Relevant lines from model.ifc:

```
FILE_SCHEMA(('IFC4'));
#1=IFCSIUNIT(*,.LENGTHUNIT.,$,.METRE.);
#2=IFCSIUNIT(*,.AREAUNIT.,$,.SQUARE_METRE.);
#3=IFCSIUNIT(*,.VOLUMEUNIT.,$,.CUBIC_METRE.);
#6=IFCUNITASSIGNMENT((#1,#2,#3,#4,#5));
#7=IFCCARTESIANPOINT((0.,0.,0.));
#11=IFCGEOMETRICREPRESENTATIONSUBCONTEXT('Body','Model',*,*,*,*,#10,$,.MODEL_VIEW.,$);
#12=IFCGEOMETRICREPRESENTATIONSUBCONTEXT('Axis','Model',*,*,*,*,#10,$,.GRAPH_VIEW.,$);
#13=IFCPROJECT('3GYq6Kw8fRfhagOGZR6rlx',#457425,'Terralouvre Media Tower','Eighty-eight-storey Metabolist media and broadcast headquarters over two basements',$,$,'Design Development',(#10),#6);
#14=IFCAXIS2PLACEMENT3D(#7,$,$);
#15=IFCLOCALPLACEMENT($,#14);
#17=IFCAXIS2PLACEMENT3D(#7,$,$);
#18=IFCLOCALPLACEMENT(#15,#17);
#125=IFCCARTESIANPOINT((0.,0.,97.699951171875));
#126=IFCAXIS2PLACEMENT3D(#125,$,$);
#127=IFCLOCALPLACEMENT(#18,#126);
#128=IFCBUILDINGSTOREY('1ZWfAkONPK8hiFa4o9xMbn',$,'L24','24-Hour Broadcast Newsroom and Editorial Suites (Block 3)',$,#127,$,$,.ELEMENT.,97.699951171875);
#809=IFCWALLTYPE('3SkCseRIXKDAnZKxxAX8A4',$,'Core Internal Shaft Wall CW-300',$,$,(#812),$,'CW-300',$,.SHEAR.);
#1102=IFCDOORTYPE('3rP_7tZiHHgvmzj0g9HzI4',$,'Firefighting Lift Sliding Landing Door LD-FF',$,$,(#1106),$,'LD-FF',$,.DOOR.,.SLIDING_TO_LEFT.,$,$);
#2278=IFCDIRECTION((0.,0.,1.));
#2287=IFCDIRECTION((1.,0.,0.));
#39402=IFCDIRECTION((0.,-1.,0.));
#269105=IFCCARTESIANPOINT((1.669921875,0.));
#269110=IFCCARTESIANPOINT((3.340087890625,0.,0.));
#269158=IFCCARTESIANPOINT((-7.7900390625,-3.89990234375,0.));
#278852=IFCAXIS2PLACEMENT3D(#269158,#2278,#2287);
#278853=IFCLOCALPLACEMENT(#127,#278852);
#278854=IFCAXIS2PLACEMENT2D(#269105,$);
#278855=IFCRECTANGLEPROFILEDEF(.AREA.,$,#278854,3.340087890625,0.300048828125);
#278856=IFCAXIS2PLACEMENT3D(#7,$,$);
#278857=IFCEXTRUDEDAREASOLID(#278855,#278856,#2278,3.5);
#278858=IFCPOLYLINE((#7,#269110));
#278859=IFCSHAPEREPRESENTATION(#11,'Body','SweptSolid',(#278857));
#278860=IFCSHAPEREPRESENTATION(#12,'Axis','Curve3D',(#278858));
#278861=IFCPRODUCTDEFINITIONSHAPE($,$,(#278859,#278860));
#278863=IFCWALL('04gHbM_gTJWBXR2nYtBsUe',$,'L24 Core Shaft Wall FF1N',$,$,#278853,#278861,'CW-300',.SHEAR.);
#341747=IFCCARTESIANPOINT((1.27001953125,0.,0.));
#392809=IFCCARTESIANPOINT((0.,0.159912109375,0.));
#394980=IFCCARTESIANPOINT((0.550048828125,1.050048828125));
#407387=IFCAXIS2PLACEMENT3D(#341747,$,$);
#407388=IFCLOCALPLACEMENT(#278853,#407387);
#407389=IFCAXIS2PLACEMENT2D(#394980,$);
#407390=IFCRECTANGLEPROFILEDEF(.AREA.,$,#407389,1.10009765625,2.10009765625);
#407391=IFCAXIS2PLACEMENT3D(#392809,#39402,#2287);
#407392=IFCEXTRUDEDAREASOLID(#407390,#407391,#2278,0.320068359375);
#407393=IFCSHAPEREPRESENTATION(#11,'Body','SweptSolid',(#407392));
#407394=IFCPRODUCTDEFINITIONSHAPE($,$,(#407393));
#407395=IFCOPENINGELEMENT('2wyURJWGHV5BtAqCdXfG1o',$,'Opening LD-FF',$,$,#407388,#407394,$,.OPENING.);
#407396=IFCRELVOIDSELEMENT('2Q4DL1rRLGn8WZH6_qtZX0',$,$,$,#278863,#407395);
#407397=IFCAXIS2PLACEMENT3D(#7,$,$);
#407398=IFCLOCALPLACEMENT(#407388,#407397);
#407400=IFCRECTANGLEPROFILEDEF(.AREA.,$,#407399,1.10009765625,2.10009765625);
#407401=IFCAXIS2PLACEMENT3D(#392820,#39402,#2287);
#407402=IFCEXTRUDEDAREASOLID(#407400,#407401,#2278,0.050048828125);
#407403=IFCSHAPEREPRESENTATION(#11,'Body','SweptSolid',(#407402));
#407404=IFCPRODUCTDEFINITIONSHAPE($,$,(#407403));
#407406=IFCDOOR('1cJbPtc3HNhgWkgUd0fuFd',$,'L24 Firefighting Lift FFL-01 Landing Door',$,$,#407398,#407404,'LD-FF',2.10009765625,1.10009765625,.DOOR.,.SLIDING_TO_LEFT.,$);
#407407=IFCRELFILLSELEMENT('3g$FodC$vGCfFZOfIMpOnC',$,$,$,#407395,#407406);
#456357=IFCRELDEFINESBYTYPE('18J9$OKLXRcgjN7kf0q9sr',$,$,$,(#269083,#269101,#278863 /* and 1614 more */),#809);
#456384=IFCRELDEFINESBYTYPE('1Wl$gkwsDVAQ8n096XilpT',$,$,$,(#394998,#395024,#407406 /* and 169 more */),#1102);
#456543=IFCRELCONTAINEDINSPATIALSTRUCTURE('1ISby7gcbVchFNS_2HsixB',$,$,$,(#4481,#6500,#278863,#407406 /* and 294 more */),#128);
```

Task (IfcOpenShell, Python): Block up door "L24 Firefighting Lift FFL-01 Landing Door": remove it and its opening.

```python
import ifcopenshell
import ifcopenshell.api.feature
import ifcopenshell.api.root
import ifcopenshell.geom
import ifcopenshell.util.shape

model = ifcopenshell.open("model.ifc")
settings = ifcopenshell.geom.settings()


def volume(element):
    """Net volume in cubic metres, openings subtracted."""
    shape = ifcopenshell.geom.create_shape(settings, element)
    return ifcopenshell.util.shape.get_volume(shape.geometry)


door = model.by_id(407406)
opening = door.FillsVoids[0].RelatingOpeningElement
wall = opening.VoidsElements[0].RelatingBuildingElement
before = volume(wall)

ifcopenshell.api.root.remove_product(model, product=door)
ifcopenshell.api.feature.remove_feature(model, feature=opening)

after = volume(wall)

print(f"wall volume {before:.3f} -> {after:.3f} m3")

model.write("model-out.ifc")
```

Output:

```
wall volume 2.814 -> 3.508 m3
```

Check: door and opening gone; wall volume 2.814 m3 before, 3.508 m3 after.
